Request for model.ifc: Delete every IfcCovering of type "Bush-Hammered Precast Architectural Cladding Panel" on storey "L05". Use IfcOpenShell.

First a look at what the model holds.

```python
import ifcopenshell
import ifcopenshell.util.element

model = ifcopenshell.open("model.ifc")
print(model.schema)
storey = next(s for s in model.by_type("IfcBuildingStorey") if s.Name == "L05")
coverings = [e for e in ifcopenshell.util.element.get_decomposition(storey) if e.is_a("IfcCovering")]
seen = {}
for e in coverings:
    element_type = ifcopenshell.util.element.get_type(e)
    name = element_type.Name if element_type not in (None, e) else None
    seen[name] = seen.get(name, 0) + 1
for name, count in sorted(seen.items(), key=str):
    print(count, "x", name)
```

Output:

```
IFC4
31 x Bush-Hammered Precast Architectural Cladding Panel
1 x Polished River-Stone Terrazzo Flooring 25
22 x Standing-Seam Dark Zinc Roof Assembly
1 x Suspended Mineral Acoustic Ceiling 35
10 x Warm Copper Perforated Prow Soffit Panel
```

```python
import ifcopenshell
import ifcopenshell.api.root
import ifcopenshell.util.element

model = ifcopenshell.open("model.ifc")

storey = next(s for s in model.by_type("IfcBuildingStorey") if s.Name == "L05")
coverings = [e for e in ifcopenshell.util.element.get_decomposition(storey) if e.is_a("IfcCovering")]
targets = [e for e in coverings if (t := ifcopenshell.util.element.get_type(e)) not in (None, e) and t.Name == "Bush-Hammered Precast Architectural Cladding Panel"]

for e in targets:
    ifcopenshell.api.root.remove_product(model, product=e)
print(len(targets), "removed")

model.write("model_updated.ifc")
```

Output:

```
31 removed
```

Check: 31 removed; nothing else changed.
